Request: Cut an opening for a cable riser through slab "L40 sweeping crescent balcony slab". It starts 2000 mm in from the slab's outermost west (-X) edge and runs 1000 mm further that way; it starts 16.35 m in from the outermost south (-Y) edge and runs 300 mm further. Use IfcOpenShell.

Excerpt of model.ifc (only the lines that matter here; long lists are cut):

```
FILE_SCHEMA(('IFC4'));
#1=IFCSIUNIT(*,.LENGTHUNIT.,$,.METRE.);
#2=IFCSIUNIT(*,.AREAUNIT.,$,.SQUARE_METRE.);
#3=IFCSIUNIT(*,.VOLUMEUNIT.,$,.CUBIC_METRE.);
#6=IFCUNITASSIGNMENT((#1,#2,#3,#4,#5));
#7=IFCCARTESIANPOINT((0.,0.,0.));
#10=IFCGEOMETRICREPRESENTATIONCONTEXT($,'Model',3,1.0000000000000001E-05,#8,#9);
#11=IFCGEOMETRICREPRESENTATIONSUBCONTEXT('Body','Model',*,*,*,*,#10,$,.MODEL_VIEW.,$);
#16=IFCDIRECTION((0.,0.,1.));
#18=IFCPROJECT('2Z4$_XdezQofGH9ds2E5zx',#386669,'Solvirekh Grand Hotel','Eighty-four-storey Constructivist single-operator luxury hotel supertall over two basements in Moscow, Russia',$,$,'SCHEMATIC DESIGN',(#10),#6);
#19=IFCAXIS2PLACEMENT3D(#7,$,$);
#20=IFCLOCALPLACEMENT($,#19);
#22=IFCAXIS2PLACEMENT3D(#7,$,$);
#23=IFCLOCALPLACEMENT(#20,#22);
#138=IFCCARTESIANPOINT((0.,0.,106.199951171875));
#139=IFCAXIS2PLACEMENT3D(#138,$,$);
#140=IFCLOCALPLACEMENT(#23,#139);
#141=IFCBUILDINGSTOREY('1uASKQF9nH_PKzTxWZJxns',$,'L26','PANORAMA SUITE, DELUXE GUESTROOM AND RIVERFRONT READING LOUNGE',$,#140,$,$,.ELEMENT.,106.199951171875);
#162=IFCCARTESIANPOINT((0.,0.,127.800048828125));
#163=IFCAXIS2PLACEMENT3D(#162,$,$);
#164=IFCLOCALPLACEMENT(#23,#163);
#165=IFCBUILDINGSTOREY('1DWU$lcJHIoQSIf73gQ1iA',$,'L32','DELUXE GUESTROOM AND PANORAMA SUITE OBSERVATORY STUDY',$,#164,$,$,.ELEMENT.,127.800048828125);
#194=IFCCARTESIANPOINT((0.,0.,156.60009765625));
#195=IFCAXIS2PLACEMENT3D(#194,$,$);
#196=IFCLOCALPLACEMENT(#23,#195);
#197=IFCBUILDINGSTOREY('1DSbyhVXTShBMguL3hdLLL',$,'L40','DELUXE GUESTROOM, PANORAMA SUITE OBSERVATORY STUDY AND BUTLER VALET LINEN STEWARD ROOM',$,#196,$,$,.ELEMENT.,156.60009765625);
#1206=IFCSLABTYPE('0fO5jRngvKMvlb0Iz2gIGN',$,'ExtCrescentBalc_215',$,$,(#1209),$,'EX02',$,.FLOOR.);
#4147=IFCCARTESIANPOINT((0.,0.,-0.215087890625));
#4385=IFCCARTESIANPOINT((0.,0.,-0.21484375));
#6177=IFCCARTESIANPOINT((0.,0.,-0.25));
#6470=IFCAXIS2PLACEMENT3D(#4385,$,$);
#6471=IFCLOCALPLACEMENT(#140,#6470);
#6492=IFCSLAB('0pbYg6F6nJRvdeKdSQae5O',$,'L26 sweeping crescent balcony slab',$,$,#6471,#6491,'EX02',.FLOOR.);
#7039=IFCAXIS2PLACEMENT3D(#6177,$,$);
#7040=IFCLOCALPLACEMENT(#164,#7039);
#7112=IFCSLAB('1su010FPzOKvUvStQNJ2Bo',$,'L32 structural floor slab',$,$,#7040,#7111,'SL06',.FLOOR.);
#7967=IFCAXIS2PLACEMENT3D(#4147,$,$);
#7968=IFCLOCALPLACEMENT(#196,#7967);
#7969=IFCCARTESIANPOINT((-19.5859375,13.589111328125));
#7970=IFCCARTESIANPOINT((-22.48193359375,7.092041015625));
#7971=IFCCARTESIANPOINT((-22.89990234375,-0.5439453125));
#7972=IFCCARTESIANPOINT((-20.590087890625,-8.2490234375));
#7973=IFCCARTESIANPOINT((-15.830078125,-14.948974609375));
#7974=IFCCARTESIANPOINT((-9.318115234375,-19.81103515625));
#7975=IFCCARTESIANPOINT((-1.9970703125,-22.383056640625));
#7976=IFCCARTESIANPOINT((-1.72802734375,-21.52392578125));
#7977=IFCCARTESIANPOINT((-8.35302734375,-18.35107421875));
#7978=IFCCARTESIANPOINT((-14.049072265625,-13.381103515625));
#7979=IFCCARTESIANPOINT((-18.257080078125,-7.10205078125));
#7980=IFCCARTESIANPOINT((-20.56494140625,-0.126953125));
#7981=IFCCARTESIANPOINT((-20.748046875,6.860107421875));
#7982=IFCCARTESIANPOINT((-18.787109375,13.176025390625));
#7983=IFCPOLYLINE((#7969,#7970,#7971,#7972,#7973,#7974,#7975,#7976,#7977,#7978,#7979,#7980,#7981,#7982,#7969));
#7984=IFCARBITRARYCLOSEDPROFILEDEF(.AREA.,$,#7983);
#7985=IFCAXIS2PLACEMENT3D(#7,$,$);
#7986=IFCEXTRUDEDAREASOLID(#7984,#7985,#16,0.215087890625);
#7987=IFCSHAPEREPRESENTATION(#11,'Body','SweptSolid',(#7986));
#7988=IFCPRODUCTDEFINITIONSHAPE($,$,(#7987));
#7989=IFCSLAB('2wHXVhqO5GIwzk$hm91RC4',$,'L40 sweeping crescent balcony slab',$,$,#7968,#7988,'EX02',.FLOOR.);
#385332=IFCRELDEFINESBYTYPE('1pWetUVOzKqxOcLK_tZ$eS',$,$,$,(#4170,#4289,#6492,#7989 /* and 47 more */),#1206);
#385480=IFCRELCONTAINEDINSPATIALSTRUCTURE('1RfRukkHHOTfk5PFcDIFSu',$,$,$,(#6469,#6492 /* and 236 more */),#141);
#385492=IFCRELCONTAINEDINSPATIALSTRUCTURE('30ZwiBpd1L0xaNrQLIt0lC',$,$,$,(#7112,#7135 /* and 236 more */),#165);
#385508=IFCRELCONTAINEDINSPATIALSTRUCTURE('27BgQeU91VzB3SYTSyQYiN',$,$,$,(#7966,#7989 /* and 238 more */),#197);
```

```python
import numpy as np
import ifcopenshell
import ifcopenshell.api.feature
import ifcopenshell.api.geometry
import ifcopenshell.api.root
import ifcopenshell.geom
import ifcopenshell.util.placement
import ifcopenshell.util.representation
import ifcopenshell.util.shape
import ifcopenshell.util.unit

model = ifcopenshell.open("model.ifc")
unit_scale = ifcopenshell.util.unit.calculate_unit_scale(model)
settings = ifcopenshell.geom.settings()


def volume(element):
    """Net volume in cubic metres, openings subtracted."""
    shape = ifcopenshell.geom.create_shape(settings, element)
    return ifcopenshell.util.shape.get_volume(shape.geometry)


slab = model.by_id(7989)
before = volume(slab)

# Extent in the slab's own axes, in metres. The edges named are its -X and -Y sides.
slab_shape = ifcopenshell.geom.create_shape(settings, slab)
vertices = ifcopenshell.util.shape.get_vertices(slab_shape.geometry)
x_min, y_min, bottom = vertices.min(axis=0)
top = vertices[:, 2].max()

opening = ifcopenshell.api.root.create_entity(model, ifc_class="IfcOpeningElement", name="Cable riser opening", predefined_type="OPENING")
context = ifcopenshell.util.representation.get_context(model, "Model", "Body", "MODEL_VIEW")
width, depth = 1, 0.3
outline = [(0.0, 0.0), (width, 0.0), (width, depth), (0.0, depth), (0.0, 0.0)]
# Overshoot both faces by 50 mm so the cut is clean.
shape = ifcopenshell.api.geometry.add_slab_representation(
    model, context=context, depth=top - bottom + 0.1, polyline=outline
)
ifcopenshell.api.geometry.assign_representation(model, product=opening, representation=shape)

matrix = ifcopenshell.util.placement.get_local_placement(slab.ObjectPlacement)
matrix[:, 3] = matrix @ np.append(np.array([x_min + 2, y_min + 16.35, bottom - 0.05]) / unit_scale, 1.0)
ifcopenshell.api.geometry.edit_object_placement(model, product=opening, matrix=matrix, is_si=False)
ifcopenshell.api.feature.add_feature(model, feature=opening, element=slab)

after = volume(slab)

print(f"slab volume {before:.3f} -> {after:.3f} m3")

model.write("model_rev.ifc")
```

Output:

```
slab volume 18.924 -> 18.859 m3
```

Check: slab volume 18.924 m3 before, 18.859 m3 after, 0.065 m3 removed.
